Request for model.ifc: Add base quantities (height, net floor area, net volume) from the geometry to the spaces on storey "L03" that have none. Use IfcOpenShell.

First a look at what the model holds.

```python
import ifcopenshell
import ifcopenshell.util.element
import ifcopenshell.util.unit

model = ifcopenshell.open("model.ifc")
print(model.schema)
for unit_type in ("LENGTHUNIT", "AREAUNIT", "VOLUMEUNIT"):
    print(unit_type, ifcopenshell.util.unit.calculate_unit_scale(model, unit_type))
storey = next(s for s in model.by_type("IfcBuildingStorey") if s.Name == "L03")
spaces = [e for e in ifcopenshell.util.element.get_decomposition(storey) if e.is_a("IfcSpace")]
for e in sorted(spaces, key=lambda e: e.id()):
    print(e.id(), e.is_a(), e.Name, list(ifcopenshell.util.element.get_psets(e, qtos_only=True)), sep=" | ")
```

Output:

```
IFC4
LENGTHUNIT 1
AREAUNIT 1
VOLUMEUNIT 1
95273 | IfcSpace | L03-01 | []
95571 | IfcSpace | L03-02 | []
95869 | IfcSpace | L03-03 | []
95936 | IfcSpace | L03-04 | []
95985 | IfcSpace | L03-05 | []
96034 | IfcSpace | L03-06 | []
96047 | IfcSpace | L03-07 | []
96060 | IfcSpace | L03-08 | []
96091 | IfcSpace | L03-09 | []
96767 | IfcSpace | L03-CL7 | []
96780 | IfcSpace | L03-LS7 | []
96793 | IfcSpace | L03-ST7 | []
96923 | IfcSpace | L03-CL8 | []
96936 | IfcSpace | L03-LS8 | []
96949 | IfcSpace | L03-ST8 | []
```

```python
import ifcopenshell
import ifcopenshell.api.pset
import ifcopenshell.geom
import ifcopenshell.util.element
import ifcopenshell.util.shape
import ifcopenshell.util.unit

model = ifcopenshell.open("model.ifc")
unit_scale = ifcopenshell.util.unit.calculate_unit_scale(model)
area_scale = ifcopenshell.util.unit.calculate_unit_scale(model, "AREAUNIT")
volume_scale = ifcopenshell.util.unit.calculate_unit_scale(model, "VOLUMEUNIT")
settings = ifcopenshell.geom.settings()

storey = next(s for s in model.by_type("IfcBuildingStorey") if s.Name == "L03")
spaces = [e for e in ifcopenshell.util.element.get_decomposition(storey) if e.is_a("IfcSpace")]

for e in sorted(spaces, key=lambda e: e.id()):
    if ifcopenshell.util.element.get_psets(e, qtos_only=True, should_inherit=False):
        continue
    # Geometry comes back in metres, in the element's own axes.
    shape = ifcopenshell.geom.create_shape(settings, e)
    values = {
        "Height": ifcopenshell.util.shape.get_z(shape.geometry) / unit_scale,
        "NetFloorArea": ifcopenshell.util.shape.get_footprint_area(shape.geometry) / area_scale,
        "NetVolume": ifcopenshell.util.shape.get_volume(shape.geometry) / volume_scale,
    }
    qto = ifcopenshell.api.pset.add_qto(model, product=e, name="Qto_SpaceBaseQuantities")
    ifcopenshell.api.pset.edit_qto(model, qto=qto, properties=values)
    print(e.id(), {k: round(v, 3) for k, v in values.items()})

model.write("model-out.ifc")
```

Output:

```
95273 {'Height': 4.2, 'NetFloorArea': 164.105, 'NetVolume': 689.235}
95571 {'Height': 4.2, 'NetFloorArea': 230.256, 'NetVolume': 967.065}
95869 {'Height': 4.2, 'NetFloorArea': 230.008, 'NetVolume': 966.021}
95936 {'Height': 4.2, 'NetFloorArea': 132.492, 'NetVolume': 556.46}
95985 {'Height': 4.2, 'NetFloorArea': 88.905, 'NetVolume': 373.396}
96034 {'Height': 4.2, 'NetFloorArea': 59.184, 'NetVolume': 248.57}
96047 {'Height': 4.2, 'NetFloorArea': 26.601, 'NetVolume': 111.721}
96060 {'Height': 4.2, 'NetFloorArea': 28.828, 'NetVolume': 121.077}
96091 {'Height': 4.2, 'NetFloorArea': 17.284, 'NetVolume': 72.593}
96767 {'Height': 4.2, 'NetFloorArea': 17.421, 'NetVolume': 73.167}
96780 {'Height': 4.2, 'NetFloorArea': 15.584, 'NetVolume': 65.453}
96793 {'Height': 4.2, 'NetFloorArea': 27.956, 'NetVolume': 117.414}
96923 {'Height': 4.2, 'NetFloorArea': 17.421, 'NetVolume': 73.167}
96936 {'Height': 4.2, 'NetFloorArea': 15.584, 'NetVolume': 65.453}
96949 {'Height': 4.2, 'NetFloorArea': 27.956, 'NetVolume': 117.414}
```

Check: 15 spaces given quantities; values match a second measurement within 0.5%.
